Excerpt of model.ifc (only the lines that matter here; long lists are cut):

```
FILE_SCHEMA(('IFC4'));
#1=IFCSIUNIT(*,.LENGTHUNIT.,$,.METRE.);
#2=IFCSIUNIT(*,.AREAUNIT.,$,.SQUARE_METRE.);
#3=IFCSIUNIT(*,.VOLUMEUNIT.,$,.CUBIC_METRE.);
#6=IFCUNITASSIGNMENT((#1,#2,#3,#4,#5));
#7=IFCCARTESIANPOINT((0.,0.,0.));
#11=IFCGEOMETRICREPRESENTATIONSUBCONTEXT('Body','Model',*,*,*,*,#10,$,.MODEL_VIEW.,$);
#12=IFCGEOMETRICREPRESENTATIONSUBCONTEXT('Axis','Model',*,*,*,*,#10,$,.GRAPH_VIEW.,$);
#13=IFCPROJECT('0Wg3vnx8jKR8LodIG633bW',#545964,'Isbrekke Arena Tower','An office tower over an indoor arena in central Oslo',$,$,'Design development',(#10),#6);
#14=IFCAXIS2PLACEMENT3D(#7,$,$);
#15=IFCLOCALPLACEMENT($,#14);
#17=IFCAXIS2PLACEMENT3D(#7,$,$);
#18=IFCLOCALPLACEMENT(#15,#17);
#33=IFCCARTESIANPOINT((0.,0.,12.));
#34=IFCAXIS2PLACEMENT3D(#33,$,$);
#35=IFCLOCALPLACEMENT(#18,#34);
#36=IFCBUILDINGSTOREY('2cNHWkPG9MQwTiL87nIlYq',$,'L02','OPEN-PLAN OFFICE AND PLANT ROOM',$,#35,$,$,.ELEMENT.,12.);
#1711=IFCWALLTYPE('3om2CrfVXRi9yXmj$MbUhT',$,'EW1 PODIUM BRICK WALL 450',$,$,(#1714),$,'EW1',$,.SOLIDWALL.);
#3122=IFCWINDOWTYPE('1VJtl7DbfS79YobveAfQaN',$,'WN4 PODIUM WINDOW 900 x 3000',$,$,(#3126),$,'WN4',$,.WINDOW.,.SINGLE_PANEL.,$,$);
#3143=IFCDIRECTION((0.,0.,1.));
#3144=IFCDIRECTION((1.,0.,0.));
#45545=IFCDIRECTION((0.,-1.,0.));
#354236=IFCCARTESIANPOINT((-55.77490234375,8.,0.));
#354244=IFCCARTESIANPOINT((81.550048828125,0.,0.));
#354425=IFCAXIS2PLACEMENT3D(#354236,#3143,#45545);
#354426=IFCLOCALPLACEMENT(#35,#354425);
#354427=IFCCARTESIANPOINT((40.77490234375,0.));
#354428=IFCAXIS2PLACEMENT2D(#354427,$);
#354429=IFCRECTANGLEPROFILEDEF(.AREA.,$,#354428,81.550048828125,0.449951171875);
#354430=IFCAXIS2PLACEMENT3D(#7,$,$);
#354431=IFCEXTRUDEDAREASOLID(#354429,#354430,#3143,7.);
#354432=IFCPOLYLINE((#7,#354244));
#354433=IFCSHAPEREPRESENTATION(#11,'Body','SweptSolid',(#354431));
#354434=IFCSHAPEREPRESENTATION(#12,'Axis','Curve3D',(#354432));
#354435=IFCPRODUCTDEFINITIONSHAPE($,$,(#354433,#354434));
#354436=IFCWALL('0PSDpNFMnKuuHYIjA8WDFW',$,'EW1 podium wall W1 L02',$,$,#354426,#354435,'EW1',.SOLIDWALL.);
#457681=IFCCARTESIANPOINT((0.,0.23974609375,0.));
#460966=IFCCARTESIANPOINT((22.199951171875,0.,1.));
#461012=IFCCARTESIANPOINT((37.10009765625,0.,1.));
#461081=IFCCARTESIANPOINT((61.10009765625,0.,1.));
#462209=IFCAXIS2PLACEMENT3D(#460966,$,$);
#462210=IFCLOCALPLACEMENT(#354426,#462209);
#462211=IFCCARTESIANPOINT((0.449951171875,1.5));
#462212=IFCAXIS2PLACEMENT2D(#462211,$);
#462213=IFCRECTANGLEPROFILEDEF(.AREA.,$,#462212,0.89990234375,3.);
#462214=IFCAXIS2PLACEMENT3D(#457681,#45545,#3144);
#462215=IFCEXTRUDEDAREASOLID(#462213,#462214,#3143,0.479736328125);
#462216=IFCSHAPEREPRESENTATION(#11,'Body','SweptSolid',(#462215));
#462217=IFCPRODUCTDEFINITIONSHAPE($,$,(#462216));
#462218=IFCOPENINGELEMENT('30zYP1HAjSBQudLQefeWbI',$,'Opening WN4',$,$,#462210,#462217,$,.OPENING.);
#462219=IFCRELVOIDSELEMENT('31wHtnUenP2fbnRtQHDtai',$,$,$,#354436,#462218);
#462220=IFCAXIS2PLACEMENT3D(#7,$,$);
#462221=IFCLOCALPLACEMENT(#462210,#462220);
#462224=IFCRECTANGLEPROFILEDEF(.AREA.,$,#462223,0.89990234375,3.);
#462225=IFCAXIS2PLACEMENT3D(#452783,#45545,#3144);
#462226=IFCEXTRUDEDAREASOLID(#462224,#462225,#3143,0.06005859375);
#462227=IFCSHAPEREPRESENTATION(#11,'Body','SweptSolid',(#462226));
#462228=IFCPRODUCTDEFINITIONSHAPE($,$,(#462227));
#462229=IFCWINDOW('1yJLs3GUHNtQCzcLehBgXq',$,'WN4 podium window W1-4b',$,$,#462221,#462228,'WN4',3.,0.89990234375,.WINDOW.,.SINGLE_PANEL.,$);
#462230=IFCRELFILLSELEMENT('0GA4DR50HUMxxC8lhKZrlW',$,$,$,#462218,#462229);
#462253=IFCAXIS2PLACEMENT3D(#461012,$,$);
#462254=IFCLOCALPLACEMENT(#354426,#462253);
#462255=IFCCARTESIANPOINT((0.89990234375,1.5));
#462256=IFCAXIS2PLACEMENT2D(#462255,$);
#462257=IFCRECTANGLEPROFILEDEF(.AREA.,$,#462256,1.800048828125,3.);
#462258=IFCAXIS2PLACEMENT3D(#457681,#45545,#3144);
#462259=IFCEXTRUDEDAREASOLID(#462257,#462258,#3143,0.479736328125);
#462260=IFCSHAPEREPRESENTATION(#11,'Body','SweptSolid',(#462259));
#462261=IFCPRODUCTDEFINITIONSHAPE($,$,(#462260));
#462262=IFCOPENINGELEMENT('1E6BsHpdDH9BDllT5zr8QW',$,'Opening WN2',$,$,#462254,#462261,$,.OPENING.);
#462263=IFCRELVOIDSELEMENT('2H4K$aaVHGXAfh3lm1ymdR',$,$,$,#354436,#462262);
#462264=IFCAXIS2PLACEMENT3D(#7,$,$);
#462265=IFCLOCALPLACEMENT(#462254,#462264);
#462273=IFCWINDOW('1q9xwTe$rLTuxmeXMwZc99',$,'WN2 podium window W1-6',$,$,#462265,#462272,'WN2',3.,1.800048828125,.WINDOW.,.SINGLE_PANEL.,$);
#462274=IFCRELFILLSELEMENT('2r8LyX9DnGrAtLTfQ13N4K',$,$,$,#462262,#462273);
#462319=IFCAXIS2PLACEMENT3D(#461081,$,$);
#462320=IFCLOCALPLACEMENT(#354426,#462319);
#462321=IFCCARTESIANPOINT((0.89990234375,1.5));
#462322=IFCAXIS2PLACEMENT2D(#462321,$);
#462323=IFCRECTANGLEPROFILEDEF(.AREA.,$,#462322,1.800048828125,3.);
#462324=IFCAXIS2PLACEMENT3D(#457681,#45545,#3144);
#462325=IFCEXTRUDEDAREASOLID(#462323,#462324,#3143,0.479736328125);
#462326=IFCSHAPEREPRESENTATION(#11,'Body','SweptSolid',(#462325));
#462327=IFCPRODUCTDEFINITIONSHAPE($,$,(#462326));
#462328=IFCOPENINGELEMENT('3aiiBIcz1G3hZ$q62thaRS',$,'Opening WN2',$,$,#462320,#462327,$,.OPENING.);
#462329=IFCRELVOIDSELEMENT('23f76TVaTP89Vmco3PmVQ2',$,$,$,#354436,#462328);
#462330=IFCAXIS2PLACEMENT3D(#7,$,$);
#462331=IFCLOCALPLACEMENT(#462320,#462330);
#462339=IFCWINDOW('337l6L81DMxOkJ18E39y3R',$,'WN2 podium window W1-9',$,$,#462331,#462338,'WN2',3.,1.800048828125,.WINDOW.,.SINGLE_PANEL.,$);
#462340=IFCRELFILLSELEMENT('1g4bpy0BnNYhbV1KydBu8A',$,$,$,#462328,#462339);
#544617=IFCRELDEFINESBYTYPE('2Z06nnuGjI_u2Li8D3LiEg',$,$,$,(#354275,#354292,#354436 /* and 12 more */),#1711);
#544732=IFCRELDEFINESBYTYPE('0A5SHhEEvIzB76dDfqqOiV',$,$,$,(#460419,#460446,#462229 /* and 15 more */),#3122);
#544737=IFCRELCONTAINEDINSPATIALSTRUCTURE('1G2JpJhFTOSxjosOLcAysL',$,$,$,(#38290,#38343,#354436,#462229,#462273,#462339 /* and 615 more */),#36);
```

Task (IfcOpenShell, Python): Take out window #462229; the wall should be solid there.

```python
import ifcopenshell
import ifcopenshell.api.feature
import ifcopenshell.api.root
import ifcopenshell.geom
import ifcopenshell.util.shape

model = ifcopenshell.open("model.ifc")
settings = ifcopenshell.geom.settings()


def volume(element):
    """Net volume in cubic metres, openings subtracted."""
    shape = ifcopenshell.geom.create_shape(settings, element)
    return ifcopenshell.util.shape.get_volume(shape.geometry)


window = model.by_guid("1yJLs3GUHNtQCzcLehBgXq")
opening = window.FillsVoids[0].RelatingOpeningElement
wall = opening.VoidsElements[0].RelatingBuildingElement
before = volume(wall)

ifcopenshell.api.root.remove_product(model, product=window)
ifcopenshell.api.feature.remove_feature(model, feature=opening)

after = volume(wall)

print(f"wall volume {before:.3f} -> {after:.3f} m3")

model.write("model_rev.ifc")
```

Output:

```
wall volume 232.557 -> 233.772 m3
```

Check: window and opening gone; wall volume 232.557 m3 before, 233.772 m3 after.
